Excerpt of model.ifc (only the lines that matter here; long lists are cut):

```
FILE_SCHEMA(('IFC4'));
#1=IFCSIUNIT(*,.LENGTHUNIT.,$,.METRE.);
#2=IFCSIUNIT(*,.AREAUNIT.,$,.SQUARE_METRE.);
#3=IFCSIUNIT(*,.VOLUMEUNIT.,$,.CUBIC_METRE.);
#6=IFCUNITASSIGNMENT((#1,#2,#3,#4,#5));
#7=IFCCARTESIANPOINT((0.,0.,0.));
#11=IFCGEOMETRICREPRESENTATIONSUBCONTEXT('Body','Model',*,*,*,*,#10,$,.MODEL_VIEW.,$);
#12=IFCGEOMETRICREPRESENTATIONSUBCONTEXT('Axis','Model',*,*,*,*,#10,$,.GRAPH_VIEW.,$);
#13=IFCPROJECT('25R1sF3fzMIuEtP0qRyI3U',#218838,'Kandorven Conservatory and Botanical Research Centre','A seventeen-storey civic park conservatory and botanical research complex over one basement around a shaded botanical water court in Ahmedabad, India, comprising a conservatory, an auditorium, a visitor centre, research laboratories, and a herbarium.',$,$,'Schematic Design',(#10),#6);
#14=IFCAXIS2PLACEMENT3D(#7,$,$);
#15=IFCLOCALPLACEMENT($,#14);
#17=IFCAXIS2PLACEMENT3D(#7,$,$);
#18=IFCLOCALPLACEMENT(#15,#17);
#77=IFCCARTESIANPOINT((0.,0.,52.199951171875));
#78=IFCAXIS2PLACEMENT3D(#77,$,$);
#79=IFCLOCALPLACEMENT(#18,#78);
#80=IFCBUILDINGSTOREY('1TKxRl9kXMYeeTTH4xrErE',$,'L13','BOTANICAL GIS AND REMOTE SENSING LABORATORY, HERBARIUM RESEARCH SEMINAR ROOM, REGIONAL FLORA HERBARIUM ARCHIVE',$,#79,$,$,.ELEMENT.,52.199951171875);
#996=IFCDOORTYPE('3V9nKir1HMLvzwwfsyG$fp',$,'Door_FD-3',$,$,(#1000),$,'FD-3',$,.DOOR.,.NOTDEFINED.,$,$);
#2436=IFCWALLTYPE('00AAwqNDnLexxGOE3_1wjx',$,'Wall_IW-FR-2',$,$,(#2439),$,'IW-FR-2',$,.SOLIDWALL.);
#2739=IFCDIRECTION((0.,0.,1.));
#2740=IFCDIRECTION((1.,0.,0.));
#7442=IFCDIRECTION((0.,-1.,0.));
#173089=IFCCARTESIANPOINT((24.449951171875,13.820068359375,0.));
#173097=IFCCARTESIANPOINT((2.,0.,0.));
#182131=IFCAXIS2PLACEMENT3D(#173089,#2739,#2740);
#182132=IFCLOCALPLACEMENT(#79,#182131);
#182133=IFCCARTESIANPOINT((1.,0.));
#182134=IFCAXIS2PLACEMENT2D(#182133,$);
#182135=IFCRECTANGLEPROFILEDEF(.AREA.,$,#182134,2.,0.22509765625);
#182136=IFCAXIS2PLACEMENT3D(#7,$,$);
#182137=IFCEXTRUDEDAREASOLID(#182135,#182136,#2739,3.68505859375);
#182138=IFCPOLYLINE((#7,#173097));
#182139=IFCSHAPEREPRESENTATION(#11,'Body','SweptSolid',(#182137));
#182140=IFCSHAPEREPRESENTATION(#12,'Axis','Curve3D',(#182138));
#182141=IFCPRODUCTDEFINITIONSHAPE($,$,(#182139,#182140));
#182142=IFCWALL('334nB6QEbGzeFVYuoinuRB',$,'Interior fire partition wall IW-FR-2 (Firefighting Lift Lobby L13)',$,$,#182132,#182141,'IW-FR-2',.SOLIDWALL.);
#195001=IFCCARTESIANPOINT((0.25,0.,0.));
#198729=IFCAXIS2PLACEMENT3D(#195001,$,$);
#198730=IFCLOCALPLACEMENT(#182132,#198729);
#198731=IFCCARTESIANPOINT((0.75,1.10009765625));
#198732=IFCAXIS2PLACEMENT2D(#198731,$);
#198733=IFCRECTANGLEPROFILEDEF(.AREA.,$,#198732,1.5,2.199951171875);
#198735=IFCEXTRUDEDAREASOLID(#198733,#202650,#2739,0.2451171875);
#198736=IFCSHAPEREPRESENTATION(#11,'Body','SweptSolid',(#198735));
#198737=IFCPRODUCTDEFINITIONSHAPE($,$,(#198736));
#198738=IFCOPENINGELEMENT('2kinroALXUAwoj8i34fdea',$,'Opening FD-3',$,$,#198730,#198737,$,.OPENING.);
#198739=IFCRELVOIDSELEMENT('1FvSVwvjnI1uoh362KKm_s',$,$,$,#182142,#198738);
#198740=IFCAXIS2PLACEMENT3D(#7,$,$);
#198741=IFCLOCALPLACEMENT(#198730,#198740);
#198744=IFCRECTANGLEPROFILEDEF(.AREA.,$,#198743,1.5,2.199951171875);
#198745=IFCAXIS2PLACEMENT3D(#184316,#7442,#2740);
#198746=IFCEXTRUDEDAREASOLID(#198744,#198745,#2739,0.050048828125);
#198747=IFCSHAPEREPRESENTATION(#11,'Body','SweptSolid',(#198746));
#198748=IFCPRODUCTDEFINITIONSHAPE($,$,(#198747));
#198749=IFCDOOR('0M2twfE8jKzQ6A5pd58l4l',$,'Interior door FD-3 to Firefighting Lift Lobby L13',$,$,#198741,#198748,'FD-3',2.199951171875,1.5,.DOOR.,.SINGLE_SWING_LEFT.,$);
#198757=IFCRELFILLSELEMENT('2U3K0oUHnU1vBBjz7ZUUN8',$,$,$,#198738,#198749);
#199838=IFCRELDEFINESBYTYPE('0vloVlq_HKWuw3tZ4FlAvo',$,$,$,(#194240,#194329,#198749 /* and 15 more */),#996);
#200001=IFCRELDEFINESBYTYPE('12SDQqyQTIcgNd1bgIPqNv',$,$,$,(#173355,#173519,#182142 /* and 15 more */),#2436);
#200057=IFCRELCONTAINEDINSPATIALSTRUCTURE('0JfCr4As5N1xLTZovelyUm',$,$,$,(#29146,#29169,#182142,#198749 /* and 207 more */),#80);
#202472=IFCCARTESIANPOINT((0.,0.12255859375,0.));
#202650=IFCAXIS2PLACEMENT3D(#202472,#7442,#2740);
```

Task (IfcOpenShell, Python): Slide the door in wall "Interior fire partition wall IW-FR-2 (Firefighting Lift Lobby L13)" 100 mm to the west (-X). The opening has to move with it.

```python
import ifcopenshell
import ifcopenshell.api.geometry
import ifcopenshell.util.placement
import ifcopenshell.util.unit

model = ifcopenshell.open("model.ifc")
unit_scale = ifcopenshell.util.unit.calculate_unit_scale(model)

door = model.by_id(198749)
opening = door.FillsVoids[0].RelatingOpeningElement
wall = opening.VoidsElements[0].RelatingBuildingElement

wall_matrix = ifcopenshell.util.placement.get_local_placement(wall.ObjectPlacement)
shift = wall_matrix[:3, 0] * -0.1 / unit_scale
before = ifcopenshell.util.placement.get_local_placement(door.ObjectPlacement)[:3, 3].copy()

# The door is placed relative to its opening, so it follows when the opening moves.
matrix = ifcopenshell.util.placement.get_local_placement(opening.ObjectPlacement)
matrix[:3, 3] += shift
ifcopenshell.api.geometry.edit_object_placement(
    model, product=opening, matrix=matrix, is_si=False, should_transform_children=True
)

after = ifcopenshell.util.placement.get_local_placement(door.ObjectPlacement)[:3, 3]
print("door moved by", (after - before).round(3) + 0.0)

model.write("model_v2.ifc")
```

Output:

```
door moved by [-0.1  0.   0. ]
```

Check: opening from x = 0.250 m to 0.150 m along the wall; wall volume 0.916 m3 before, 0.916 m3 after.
